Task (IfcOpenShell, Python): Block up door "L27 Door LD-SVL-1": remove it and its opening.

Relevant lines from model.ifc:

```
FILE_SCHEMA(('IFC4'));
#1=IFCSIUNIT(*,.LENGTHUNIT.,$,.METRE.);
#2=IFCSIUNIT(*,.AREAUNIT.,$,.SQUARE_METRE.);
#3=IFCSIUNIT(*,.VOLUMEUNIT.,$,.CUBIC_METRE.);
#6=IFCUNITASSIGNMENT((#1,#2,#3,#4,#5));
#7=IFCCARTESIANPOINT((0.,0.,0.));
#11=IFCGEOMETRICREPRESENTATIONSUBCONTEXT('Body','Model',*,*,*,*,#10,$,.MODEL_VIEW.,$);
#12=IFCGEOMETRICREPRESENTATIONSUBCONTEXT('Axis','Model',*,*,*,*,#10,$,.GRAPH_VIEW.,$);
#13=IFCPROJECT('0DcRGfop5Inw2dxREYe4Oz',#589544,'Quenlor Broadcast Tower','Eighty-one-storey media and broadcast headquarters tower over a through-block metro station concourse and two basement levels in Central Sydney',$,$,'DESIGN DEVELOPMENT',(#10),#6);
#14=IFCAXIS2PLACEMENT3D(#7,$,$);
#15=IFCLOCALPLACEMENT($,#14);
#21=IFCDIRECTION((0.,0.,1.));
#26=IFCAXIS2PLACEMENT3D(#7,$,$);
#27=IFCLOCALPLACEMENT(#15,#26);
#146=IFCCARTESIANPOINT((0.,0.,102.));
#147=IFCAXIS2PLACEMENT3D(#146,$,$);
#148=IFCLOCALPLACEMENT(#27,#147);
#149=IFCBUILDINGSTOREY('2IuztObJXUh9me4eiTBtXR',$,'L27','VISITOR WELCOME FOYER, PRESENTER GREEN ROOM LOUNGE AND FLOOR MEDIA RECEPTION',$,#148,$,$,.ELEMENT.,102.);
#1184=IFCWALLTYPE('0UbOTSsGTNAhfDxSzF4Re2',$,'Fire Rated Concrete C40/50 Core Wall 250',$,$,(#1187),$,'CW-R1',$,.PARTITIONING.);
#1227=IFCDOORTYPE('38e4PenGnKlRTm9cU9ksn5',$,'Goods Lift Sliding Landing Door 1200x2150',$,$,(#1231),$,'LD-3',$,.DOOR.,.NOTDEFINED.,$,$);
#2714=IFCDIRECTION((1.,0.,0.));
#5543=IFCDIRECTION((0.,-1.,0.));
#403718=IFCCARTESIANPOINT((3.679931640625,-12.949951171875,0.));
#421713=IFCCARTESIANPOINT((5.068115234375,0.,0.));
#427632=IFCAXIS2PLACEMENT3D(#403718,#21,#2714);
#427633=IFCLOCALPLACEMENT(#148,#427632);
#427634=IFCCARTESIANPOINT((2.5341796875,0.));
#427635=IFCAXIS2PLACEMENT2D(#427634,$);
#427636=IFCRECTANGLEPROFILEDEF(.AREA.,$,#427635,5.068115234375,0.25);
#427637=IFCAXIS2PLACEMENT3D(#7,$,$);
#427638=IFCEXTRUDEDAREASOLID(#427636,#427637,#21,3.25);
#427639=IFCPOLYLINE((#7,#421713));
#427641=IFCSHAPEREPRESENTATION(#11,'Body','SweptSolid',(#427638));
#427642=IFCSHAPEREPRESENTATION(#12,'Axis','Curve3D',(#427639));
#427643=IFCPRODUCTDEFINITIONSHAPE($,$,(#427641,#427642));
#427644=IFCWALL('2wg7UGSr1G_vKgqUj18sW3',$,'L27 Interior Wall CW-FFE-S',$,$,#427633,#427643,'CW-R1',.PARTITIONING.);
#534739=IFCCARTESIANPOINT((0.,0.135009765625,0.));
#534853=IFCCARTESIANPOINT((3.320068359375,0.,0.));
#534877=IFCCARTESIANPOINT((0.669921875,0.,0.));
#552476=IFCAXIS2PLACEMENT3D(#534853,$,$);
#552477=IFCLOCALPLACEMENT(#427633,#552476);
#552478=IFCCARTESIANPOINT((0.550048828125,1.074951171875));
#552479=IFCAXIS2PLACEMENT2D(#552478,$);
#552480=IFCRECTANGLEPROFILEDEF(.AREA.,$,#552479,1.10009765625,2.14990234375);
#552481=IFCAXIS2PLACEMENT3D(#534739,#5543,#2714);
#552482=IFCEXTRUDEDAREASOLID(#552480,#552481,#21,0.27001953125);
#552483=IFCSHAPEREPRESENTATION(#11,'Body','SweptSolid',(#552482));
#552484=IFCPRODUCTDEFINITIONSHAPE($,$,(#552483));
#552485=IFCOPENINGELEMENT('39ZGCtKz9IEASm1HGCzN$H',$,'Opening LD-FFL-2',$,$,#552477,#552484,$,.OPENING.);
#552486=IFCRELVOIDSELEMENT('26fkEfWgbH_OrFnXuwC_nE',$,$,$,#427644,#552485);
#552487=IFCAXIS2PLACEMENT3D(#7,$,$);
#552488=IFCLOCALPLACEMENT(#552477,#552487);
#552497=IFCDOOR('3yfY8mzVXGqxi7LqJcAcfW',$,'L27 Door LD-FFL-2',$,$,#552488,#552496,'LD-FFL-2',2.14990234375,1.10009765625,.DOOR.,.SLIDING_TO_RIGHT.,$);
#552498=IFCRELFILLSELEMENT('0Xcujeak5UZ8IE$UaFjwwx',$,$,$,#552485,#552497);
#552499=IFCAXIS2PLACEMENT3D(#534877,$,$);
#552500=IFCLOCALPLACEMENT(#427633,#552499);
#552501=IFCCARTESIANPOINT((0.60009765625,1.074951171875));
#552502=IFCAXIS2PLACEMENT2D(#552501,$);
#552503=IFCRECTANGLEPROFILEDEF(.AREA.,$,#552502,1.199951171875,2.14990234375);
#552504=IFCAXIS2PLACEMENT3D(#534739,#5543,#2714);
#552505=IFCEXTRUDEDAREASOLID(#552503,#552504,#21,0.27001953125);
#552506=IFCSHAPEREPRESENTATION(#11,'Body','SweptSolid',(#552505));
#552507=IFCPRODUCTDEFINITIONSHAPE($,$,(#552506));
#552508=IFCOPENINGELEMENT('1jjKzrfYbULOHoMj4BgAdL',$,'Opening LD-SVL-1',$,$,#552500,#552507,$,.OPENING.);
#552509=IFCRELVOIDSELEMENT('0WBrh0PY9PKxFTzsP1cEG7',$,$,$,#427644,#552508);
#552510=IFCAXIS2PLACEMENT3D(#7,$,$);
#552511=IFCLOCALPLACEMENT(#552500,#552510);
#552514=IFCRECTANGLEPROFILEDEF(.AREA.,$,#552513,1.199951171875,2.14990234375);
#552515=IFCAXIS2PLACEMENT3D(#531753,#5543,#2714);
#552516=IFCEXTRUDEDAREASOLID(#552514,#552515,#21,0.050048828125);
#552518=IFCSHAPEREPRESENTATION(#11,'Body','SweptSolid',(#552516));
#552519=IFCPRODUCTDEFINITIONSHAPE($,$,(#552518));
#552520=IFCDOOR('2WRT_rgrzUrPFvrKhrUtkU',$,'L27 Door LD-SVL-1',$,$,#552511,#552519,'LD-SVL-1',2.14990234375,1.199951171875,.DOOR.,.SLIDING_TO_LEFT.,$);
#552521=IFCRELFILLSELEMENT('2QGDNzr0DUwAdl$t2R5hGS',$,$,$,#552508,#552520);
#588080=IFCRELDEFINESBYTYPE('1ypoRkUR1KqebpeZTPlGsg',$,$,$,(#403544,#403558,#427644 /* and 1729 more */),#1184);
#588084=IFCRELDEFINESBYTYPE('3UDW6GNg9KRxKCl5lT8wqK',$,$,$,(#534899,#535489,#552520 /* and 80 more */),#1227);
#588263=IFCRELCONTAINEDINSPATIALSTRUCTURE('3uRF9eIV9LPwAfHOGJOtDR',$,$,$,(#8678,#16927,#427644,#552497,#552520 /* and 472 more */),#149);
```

```python
import ifcopenshell
import ifcopenshell.api.feature
import ifcopenshell.api.root
import ifcopenshell.geom
import ifcopenshell.util.shape

model = ifcopenshell.open("model.ifc")
settings = ifcopenshell.geom.settings()


def volume(element):
    """Net volume in cubic metres, openings subtracted."""
    shape = ifcopenshell.geom.create_shape(settings, element)
    return ifcopenshell.util.shape.get_volume(shape.geometry)


door = model.by_guid("2WRT_rgrzUrPFvrKhrUtkU")
opening = door.FillsVoids[0].RelatingOpeningElement
wall = opening.VoidsElements[0].RelatingBuildingElement
before = volume(wall)

ifcopenshell.api.root.remove_product(model, product=door)
ifcopenshell.api.feature.remove_feature(model, feature=opening)

after = volume(wall)

print(f"wall volume {before:.3f} -> {after:.3f} m3")

model.write("model_edited.ifc")
```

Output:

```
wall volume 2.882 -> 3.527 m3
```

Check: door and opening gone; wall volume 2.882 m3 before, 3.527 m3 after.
